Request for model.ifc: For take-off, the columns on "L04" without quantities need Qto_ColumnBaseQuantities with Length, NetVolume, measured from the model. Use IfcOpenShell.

First a look at what the model holds.

```python
import ifcopenshell
import ifcopenshell.util.element
import ifcopenshell.util.unit

model = ifcopenshell.open("model.ifc")
print(model.schema)
for unit_type in ("LENGTHUNIT", "AREAUNIT", "VOLUMEUNIT"):
    print(unit_type, ifcopenshell.util.unit.calculate_unit_scale(model, unit_type))
storey = next(s for s in model.by_type("IfcBuildingStorey") if s.Name == "L04")
columns = [e for e in ifcopenshell.util.element.get_decomposition(storey) if e.is_a("IfcColumn")]
for e in sorted(columns, key=lambda e: e.id()):
    print(e.id(), e.is_a(), e.Name, list(ifcopenshell.util.element.get_psets(e, qtos_only=True)), sep=" | ")
```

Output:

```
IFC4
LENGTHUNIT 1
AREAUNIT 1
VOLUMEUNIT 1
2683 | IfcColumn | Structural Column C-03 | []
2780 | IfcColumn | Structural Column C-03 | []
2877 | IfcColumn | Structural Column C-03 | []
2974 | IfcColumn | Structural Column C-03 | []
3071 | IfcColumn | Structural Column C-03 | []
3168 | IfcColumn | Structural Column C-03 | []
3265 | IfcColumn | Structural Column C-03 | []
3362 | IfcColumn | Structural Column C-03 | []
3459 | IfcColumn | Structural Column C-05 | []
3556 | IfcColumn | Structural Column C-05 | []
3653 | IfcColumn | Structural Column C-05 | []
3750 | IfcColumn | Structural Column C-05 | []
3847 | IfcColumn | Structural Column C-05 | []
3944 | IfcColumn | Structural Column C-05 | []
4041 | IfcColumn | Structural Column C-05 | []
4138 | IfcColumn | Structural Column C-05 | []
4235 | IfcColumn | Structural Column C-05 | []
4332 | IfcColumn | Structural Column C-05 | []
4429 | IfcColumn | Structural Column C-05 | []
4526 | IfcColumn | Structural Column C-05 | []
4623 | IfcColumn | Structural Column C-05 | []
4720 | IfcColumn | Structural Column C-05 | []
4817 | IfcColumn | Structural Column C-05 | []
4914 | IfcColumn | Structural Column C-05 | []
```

```python
import ifcopenshell
import ifcopenshell.api.pset
import ifcopenshell.geom
import ifcopenshell.util.element
import ifcopenshell.util.shape
import ifcopenshell.util.unit

model = ifcopenshell.open("model.ifc")
unit_scale = ifcopenshell.util.unit.calculate_unit_scale(model)
volume_scale = ifcopenshell.util.unit.calculate_unit_scale(model, "VOLUMEUNIT")
settings = ifcopenshell.geom.settings()

storey = next(s for s in model.by_type("IfcBuildingStorey") if s.Name == "L04")
columns = [e for e in ifcopenshell.util.element.get_decomposition(storey) if e.is_a("IfcColumn")]

for e in sorted(columns, key=lambda e: e.id()):
    if ifcopenshell.util.element.get_psets(e, qtos_only=True, should_inherit=False):
        continue
    # Geometry comes back in metres, in the element's own axes.
    shape = ifcopenshell.geom.create_shape(settings, e)
    values = {
        "Length": ifcopenshell.util.shape.get_z(shape.geometry) / unit_scale,
        "NetVolume": ifcopenshell.util.shape.get_volume(shape.geometry) / volume_scale,
    }
    qto = ifcopenshell.api.pset.add_qto(model, product=e, name="Qto_ColumnBaseQuantities")
    ifcopenshell.api.pset.edit_qto(model, qto=qto, properties=values)
    print(e.id(), {k: round(v, 3) for k, v in values.items()})

model.write("model_edited.ifc")
```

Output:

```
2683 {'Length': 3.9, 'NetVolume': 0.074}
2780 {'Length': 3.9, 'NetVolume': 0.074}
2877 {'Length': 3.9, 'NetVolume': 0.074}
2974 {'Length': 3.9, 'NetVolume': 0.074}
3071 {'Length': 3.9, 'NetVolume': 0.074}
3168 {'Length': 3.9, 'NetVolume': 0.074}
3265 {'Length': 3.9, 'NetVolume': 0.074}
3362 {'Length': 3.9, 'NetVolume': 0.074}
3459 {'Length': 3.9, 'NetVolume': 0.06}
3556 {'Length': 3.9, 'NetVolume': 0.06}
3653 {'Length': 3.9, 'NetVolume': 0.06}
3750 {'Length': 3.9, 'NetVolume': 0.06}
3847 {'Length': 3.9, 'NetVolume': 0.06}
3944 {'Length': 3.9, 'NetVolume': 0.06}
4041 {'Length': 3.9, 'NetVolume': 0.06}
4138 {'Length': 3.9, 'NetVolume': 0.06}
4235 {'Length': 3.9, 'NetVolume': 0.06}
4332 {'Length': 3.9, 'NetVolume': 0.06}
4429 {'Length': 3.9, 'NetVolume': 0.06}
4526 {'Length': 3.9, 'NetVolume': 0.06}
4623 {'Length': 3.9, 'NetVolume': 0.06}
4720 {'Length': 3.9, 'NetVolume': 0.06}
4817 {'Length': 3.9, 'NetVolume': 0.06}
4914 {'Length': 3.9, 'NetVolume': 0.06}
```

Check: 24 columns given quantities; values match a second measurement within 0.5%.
